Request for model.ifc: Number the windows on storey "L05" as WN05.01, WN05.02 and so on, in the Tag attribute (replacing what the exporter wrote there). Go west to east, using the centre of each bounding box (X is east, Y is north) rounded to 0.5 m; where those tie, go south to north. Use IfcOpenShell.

First a look at what the model holds.

```python
import ifcopenshell
import ifcopenshell.util.element
import ifcopenshell.util.placement

model = ifcopenshell.open("model.ifc")
print(model.schema)
storey = next(s for s in model.by_type("IfcBuildingStorey") if s.Name == "L05")
windows = [e for e in ifcopenshell.util.element.get_decomposition(storey) if e.is_a("IfcWindow")]
for e in sorted(windows, key=lambda e: e.id()):
    origin = ifcopenshell.util.placement.get_local_placement(e.ObjectPlacement)[:3, 3]
    print(e.id(), e.Tag, e.Name, origin.round(2) + 0.0, sep=" | ")
```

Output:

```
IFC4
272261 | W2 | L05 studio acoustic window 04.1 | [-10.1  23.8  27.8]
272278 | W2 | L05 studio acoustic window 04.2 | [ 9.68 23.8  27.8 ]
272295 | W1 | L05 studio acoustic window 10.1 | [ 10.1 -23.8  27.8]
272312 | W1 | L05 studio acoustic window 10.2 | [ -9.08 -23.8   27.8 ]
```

```python
import ifcopenshell
import ifcopenshell.geom
import ifcopenshell.util.element
import ifcopenshell.util.shape

model = ifcopenshell.open("model.ifc")
settings = ifcopenshell.geom.settings()
settings.set("use-world-coords", True)


def centre(element):
    shape = ifcopenshell.geom.create_shape(settings, element)
    return ifcopenshell.util.shape.get_bbox_centroid(shape.geometry)


storey = next(s for s in model.by_type("IfcBuildingStorey") if s.Name == "L05")
windows = [e for e in ifcopenshell.util.element.get_decomposition(storey) if e.is_a("IfcWindow")]

# Insertion points can sit at a corner or the storey origin, so sort by the geometry (in metres).
centres = {e: centre(e) for e in windows}
windows.sort(key=lambda e: (round(centres[e][0] / 0.5), centres[e][1]))

for i, e in enumerate(windows, start=1):
    number = f"WN05.{i:02d}"
    e.Tag = number
    print(e.id(), number)

model.write("model_rev.ifc")
```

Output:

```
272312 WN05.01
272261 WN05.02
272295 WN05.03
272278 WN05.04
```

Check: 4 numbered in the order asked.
